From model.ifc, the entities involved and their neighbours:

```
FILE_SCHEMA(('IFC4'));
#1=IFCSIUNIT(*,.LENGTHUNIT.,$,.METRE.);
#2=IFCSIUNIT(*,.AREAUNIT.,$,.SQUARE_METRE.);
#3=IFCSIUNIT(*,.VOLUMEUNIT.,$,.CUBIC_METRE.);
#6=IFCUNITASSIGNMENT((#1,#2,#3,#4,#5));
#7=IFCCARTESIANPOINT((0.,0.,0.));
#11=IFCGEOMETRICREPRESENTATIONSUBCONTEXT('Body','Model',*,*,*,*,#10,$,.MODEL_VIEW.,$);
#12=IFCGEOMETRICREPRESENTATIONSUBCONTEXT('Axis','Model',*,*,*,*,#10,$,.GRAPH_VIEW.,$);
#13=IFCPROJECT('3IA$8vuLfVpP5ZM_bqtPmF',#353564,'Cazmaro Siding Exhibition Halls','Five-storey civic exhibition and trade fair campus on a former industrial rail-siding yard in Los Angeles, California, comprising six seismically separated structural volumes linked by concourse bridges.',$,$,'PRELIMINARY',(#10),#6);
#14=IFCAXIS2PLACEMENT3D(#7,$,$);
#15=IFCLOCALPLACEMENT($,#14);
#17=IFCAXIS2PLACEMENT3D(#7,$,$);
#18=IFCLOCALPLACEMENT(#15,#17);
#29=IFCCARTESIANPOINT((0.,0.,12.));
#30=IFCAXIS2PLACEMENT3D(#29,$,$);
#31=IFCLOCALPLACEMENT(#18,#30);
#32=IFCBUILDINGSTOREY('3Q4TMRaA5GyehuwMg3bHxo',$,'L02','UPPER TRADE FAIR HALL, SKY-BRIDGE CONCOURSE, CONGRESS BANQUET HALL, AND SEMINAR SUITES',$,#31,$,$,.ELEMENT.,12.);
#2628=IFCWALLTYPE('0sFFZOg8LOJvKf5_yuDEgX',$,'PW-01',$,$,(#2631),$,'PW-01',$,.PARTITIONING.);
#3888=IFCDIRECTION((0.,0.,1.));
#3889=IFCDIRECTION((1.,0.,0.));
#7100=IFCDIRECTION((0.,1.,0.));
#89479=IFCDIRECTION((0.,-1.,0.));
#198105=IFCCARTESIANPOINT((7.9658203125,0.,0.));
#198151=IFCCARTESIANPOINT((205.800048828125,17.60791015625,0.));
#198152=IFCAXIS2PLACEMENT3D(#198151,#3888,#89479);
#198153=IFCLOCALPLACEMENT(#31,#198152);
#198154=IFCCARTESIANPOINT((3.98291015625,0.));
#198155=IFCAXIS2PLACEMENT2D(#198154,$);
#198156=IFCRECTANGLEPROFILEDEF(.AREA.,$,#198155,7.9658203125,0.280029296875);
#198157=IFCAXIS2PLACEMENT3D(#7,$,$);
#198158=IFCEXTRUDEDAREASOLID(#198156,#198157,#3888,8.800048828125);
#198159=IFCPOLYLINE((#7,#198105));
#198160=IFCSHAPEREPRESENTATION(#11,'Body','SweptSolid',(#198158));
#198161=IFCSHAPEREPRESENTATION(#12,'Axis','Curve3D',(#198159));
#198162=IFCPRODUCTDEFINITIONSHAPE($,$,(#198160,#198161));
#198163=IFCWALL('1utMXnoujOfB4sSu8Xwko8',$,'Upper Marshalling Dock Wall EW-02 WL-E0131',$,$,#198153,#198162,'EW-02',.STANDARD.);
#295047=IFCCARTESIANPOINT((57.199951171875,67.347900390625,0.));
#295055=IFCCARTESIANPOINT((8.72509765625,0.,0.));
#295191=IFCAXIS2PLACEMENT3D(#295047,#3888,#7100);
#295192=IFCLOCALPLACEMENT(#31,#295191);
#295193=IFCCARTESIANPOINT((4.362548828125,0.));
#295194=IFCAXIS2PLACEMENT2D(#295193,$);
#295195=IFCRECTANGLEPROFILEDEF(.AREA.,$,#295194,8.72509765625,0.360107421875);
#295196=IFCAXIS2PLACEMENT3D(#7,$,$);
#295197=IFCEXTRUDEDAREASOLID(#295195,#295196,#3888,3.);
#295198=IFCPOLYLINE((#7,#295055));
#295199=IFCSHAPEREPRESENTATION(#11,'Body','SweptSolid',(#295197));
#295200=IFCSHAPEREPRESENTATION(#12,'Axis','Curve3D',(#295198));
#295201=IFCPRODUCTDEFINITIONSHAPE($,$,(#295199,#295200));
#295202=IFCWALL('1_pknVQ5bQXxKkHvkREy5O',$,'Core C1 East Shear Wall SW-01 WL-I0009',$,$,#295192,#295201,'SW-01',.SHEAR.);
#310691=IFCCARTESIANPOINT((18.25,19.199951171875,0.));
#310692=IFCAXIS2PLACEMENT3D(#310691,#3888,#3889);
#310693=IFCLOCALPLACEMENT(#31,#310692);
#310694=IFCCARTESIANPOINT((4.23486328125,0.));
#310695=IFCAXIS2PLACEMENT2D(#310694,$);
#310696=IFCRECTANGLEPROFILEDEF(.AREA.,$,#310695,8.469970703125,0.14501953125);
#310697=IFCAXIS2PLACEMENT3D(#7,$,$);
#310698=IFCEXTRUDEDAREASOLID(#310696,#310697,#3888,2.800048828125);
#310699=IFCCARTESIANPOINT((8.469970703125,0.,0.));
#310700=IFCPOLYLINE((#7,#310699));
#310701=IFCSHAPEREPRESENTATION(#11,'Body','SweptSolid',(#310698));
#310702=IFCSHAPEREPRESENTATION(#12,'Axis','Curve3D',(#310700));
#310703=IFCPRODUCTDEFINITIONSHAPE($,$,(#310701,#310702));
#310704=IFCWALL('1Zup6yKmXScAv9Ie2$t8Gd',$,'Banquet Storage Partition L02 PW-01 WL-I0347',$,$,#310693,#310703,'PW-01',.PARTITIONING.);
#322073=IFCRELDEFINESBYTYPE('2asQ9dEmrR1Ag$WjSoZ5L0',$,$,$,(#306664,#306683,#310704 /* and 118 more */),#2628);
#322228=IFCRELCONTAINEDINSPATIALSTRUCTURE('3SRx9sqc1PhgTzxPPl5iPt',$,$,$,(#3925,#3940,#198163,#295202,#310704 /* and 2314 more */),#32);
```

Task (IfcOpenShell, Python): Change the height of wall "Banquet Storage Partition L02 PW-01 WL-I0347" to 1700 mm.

```python
import ifcopenshell
import ifcopenshell.geom
import ifcopenshell.util.representation
import ifcopenshell.util.shape

model = ifcopenshell.open("model.ifc")
settings = ifcopenshell.geom.settings()


def volume(element):
    """Net volume in cubic metres, openings subtracted."""
    shape = ifcopenshell.geom.create_shape(settings, element)
    return ifcopenshell.util.shape.get_volume(shape.geometry)


wall = model.by_guid("1Zup6yKmXScAv9Ie2$t8Gd")
before = volume(wall)

body = ifcopenshell.util.representation.get_representation(wall, "Model", "Body")
solid = body.Items[0]
old_height = solid.Depth
solid.Depth = 1.7
after = volume(wall)

print(f"height {old_height:g} -> {solid.Depth:g}, volume {before:.3f} -> {after:.3f} m3")

model.write("model-out.ifc")
```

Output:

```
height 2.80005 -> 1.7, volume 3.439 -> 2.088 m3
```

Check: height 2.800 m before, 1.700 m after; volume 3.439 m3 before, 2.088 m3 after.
